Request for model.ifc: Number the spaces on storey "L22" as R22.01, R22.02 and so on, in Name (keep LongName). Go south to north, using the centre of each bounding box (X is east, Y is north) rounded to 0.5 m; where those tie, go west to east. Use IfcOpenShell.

First a look at what the model holds.

```python
import ifcopenshell
import ifcopenshell.util.element
import ifcopenshell.util.placement

model = ifcopenshell.open("model.ifc")
print(model.schema)
storey = next(s for s in model.by_type("IfcBuildingStorey") if s.Name == "L22")
spaces = [e for e in ifcopenshell.util.element.get_decomposition(storey) if e.is_a("IfcSpace")]
for e in sorted(spaces, key=lambda e: e.id()):
    origin = ifcopenshell.util.placement.get_local_placement(e.ObjectPlacement)[:3, 3]
    print(e.id(), e.Name, e.LongName, origin.round(2) + 0.0, sep=" | ")
```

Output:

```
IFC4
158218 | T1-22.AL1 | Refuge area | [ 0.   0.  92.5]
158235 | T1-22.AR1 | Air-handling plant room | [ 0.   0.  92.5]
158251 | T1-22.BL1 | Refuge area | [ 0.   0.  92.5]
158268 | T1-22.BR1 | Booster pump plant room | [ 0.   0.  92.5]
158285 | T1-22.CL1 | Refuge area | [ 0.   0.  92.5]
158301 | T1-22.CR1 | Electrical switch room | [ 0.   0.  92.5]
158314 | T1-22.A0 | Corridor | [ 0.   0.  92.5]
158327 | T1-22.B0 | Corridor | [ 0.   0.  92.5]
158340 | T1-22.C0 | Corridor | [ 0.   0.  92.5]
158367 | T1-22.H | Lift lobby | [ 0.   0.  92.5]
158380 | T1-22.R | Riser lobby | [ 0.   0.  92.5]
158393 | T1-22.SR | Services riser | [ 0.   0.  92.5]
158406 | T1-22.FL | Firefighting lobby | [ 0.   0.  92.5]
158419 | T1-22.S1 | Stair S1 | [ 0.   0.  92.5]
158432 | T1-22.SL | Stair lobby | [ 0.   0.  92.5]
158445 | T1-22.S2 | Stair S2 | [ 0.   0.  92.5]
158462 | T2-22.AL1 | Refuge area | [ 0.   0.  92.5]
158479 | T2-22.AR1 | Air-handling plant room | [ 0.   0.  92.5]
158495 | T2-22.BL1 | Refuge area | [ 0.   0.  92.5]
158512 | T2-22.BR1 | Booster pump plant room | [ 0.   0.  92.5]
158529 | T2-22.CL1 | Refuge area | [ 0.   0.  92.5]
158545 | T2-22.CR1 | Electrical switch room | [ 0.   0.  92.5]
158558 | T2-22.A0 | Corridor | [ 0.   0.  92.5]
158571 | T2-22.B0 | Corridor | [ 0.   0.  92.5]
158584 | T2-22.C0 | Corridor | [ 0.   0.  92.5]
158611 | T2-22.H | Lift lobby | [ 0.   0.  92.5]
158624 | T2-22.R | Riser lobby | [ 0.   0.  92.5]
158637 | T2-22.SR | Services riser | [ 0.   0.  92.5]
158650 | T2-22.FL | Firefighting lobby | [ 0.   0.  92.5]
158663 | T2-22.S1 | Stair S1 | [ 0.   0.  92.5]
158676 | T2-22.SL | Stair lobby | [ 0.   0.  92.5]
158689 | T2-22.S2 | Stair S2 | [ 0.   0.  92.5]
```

```python
import ifcopenshell
import ifcopenshell.geom
import ifcopenshell.util.element
import ifcopenshell.util.shape

model = ifcopenshell.open("model.ifc")
settings = ifcopenshell.geom.settings()
settings.set("use-world-coords", True)


def centre(element):
    shape = ifcopenshell.geom.create_shape(settings, element)
    return ifcopenshell.util.shape.get_bbox_centroid(shape.geometry)


storey = next(s for s in model.by_type("IfcBuildingStorey") if s.Name == "L22")
spaces = [e for e in ifcopenshell.util.element.get_decomposition(storey) if e.is_a("IfcSpace")]

# Insertion points can sit at a corner or the storey origin, so sort by the geometry (in metres).
centres = {e: centre(e) for e in spaces}
spaces.sort(key=lambda e: (round(centres[e][1] / 0.5), centres[e][0]))

for i, e in enumerate(spaces, start=1):
    number = f"R22.{i:02d}"
    e.Name = number
    print(e.id(), number)

model.write("model_rev.ifc")
```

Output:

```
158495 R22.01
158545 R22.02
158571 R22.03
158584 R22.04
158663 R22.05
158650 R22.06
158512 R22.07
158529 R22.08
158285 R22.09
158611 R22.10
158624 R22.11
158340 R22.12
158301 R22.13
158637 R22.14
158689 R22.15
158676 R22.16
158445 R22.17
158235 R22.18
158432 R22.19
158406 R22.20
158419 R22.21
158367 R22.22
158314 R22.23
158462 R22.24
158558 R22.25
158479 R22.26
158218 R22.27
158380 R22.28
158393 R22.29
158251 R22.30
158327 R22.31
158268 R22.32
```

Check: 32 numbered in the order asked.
